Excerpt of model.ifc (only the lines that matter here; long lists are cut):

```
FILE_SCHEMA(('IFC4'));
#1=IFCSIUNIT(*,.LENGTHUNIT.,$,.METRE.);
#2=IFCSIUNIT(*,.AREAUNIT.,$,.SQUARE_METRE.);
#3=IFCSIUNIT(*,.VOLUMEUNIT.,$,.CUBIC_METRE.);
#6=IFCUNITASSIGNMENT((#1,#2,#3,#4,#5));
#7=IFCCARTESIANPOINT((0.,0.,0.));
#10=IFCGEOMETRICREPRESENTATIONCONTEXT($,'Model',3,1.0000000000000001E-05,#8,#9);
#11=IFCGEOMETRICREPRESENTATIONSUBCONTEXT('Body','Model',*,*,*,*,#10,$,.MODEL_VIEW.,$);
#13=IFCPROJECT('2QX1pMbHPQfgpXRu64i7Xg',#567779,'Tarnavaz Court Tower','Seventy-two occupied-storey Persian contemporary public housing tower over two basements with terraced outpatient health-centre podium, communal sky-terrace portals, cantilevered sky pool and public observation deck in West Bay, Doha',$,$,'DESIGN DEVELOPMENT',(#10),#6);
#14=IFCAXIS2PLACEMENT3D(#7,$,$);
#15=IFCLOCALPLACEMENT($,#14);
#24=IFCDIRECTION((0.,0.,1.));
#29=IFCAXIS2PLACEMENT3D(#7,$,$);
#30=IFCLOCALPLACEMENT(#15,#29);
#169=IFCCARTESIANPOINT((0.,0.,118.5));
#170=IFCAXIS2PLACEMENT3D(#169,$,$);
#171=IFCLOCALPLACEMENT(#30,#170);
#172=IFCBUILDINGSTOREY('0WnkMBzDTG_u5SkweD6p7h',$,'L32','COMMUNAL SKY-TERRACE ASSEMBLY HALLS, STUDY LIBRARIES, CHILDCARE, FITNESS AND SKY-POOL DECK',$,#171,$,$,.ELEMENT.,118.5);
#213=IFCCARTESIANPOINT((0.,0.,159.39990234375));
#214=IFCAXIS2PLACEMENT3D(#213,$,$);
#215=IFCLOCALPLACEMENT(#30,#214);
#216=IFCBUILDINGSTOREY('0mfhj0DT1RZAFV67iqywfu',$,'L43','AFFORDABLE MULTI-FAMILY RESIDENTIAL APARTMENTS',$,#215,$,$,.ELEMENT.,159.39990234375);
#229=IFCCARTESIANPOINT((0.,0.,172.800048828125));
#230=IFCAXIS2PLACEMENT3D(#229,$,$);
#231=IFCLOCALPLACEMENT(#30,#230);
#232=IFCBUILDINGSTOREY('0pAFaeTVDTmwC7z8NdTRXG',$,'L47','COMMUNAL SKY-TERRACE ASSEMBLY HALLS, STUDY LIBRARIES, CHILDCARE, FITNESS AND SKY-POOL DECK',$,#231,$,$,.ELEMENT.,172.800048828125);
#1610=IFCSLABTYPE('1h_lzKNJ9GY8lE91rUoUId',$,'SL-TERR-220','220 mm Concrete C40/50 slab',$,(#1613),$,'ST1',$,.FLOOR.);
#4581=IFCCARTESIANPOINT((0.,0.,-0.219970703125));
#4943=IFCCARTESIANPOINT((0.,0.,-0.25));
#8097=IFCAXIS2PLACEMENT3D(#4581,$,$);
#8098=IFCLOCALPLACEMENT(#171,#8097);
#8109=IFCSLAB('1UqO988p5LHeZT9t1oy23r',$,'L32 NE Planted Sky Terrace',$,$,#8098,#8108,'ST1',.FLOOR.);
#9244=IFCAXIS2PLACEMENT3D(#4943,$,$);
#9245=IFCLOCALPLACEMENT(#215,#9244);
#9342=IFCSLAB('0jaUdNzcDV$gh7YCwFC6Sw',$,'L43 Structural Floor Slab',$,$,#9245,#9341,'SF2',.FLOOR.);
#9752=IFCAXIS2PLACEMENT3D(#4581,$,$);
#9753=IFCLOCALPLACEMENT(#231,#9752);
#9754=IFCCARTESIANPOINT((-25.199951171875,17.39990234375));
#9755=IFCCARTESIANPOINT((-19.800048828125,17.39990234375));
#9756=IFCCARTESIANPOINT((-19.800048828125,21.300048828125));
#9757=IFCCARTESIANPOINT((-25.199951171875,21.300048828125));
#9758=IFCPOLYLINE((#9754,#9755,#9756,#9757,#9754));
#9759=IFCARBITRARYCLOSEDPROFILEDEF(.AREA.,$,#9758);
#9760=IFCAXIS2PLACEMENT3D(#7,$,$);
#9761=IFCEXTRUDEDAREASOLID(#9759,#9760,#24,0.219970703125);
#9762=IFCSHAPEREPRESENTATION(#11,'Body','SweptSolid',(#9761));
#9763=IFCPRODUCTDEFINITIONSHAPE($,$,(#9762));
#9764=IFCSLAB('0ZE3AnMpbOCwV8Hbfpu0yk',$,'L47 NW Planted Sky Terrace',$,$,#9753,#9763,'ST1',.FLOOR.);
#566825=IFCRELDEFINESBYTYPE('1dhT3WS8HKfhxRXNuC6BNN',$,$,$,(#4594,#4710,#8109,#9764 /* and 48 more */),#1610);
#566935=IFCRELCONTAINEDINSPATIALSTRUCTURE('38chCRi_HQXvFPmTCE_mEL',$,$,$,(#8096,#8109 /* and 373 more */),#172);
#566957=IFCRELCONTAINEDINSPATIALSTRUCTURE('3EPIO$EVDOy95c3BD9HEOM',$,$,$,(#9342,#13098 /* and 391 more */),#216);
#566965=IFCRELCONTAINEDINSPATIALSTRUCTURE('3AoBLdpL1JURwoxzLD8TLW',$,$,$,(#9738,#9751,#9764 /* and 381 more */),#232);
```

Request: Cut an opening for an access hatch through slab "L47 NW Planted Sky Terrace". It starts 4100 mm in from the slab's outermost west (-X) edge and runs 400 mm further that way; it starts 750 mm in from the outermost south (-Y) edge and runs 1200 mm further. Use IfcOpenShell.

```python
import numpy as np
import ifcopenshell
import ifcopenshell.api.feature
import ifcopenshell.api.geometry
import ifcopenshell.api.root
import ifcopenshell.geom
import ifcopenshell.util.placement
import ifcopenshell.util.representation
import ifcopenshell.util.shape
import ifcopenshell.util.unit

model = ifcopenshell.open("model.ifc")
unit_scale = ifcopenshell.util.unit.calculate_unit_scale(model)
settings = ifcopenshell.geom.settings()


def volume(element):
    """Net volume in cubic metres, openings subtracted."""
    shape = ifcopenshell.geom.create_shape(settings, element)
    return ifcopenshell.util.shape.get_volume(shape.geometry)


slab = model.by_id(9764)
before = volume(slab)

# Extent in the slab's own axes, in metres. The edges named are its -X and -Y sides.
slab_shape = ifcopenshell.geom.create_shape(settings, slab)
vertices = ifcopenshell.util.shape.get_vertices(slab_shape.geometry)
x_min, y_min, bottom = vertices.min(axis=0)
top = vertices[:, 2].max()

opening = ifcopenshell.api.root.create_entity(model, ifc_class="IfcOpeningElement", name="Access hatch opening", predefined_type="OPENING")
context = ifcopenshell.util.representation.get_context(model, "Model", "Body", "MODEL_VIEW")
width, depth = 0.4, 1.2
outline = [(0.0, 0.0), (width, 0.0), (width, depth), (0.0, depth), (0.0, 0.0)]
# Overshoot both faces by 50 mm so the cut is clean.
shape = ifcopenshell.api.geometry.add_slab_representation(
    model, context=context, depth=top - bottom + 0.1, polyline=outline
)
ifcopenshell.api.geometry.assign_representation(model, product=opening, representation=shape)

matrix = ifcopenshell.util.placement.get_local_placement(slab.ObjectPlacement)
matrix[:, 3] = matrix @ np.append(np.array([x_min + 4.1, y_min + 0.75, bottom - 0.05]) / unit_scale, 1.0)
ifcopenshell.api.geometry.edit_object_placement(model, product=opening, matrix=matrix, is_si=False)
ifcopenshell.api.feature.add_feature(model, feature=opening, element=slab)

after = volume(slab)

print(f"slab volume {before:.3f} -> {after:.3f} m3")

model.write("model_rev.ifc")
```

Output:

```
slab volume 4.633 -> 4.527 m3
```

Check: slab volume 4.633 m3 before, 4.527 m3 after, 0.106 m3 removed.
